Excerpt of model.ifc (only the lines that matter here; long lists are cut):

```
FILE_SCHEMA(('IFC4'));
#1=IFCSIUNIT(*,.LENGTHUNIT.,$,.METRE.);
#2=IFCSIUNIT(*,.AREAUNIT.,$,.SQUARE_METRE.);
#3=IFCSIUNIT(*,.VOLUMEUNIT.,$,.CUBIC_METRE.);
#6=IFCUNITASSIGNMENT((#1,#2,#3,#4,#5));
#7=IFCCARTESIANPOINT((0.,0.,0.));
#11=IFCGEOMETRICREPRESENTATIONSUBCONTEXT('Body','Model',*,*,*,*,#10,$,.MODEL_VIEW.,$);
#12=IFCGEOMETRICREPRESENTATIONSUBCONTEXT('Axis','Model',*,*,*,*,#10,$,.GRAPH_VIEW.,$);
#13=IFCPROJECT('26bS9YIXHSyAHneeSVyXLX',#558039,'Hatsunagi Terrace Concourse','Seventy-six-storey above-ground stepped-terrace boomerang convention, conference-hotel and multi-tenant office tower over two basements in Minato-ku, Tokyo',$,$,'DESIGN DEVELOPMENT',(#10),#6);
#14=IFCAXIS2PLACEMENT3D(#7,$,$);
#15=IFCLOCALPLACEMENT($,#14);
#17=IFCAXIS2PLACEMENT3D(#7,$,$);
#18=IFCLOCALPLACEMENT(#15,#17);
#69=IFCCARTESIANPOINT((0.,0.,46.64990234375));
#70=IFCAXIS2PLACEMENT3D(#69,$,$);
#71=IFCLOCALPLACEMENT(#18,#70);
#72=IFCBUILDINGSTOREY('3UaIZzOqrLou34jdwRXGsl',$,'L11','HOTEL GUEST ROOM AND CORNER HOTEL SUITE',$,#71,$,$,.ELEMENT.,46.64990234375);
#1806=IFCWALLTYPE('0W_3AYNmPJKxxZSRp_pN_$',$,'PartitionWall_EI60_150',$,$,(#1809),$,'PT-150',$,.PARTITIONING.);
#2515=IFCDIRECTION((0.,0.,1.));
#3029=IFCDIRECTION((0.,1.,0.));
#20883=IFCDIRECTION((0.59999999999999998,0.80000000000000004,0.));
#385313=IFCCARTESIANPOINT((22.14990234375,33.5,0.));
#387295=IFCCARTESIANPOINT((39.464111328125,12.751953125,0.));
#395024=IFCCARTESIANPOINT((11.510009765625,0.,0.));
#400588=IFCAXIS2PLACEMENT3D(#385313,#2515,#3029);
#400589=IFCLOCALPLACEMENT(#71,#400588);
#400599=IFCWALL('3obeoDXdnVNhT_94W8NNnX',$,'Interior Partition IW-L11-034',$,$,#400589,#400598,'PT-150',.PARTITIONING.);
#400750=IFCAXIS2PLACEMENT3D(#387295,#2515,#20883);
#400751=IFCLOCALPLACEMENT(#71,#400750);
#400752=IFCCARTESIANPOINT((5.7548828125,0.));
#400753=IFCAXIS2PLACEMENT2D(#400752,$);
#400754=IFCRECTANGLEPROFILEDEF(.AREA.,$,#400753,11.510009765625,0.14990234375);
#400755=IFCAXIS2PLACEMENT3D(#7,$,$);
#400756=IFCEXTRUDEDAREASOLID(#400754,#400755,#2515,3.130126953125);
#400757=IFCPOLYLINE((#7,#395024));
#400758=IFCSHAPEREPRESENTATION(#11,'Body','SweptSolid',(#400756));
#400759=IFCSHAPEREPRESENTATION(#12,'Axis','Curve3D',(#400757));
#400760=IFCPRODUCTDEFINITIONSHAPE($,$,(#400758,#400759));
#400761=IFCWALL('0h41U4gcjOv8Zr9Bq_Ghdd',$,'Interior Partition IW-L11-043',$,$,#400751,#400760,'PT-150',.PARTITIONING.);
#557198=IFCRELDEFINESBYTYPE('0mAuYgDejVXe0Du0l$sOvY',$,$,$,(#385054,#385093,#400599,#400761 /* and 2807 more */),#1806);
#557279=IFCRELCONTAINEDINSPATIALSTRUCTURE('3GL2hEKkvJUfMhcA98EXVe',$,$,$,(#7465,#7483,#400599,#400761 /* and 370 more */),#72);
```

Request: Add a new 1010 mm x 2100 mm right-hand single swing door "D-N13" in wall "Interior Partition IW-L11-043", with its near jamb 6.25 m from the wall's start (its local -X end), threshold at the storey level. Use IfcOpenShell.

```python
import numpy as np
import ifcopenshell
import ifcopenshell.api.feature
import ifcopenshell.api.geometry
import ifcopenshell.api.root
import ifcopenshell.api.spatial
import ifcopenshell.geom
import ifcopenshell.util.element
import ifcopenshell.util.placement
import ifcopenshell.util.representation
import ifcopenshell.util.shape
import ifcopenshell.util.unit

model = ifcopenshell.open("model.ifc")
unit_scale = ifcopenshell.util.unit.calculate_unit_scale(model)
settings = ifcopenshell.geom.settings()


def volume(element):
    """Net volume in cubic metres, openings subtracted."""
    shape = ifcopenshell.geom.create_shape(settings, element)
    return ifcopenshell.util.shape.get_volume(shape.geometry)


wall = model.by_guid("0h41U4gcjOv8Zr9Bq_Ghdd")
storey = ifcopenshell.util.element.get_container(wall, ifc_class="IfcBuildingStorey")
context = ifcopenshell.util.representation.get_context(model, "Model", "Body", "MODEL_VIEW")
before = volume(wall)

width, height, from_end, sill = 1.01, 2.1, 6.25, 0.0  # metres

# The wall runs along its own X axis, and the end named is its -X end.
wall_shape = ifcopenshell.geom.create_shape(settings, wall)
x, y, z = ifcopenshell.util.shape.get_vertices(wall_shape.geometry).T
start = x.min() + from_end
face, thickness = float(y.min()), float(y.max() - y.min())
wall_matrix = ifcopenshell.util.placement.get_local_placement(wall.ObjectPlacement)
level = ifcopenshell.util.placement.get_local_placement(storey.ObjectPlacement)[2, 3]


def in_wall(x, y):
    """Placement at x, y metres in the wall's axes, at sill height."""
    matrix = wall_matrix.copy()
    matrix[:, 3] = wall_matrix @ np.array([x / unit_scale, y / unit_scale, 0.0, 1.0])
    matrix[2, 3] = level + sill / unit_scale
    return matrix


# Opening: a box that overshoots both wall faces by 50 mm.
opening = ifcopenshell.api.root.create_entity(model, ifc_class="IfcOpeningElement", predefined_type="OPENING")
box = ifcopenshell.api.geometry.add_wall_representation(
    model, context=context, length=width, height=height, thickness=thickness + 0.1
)
ifcopenshell.api.geometry.assign_representation(model, product=opening, representation=box)
ifcopenshell.api.geometry.edit_object_placement(model, product=opening, matrix=in_wall(start, face - 0.05), is_si=False)
ifcopenshell.api.feature.add_feature(model, feature=opening, element=wall)

door = ifcopenshell.api.root.create_entity(model, ifc_class="IfcDoor", name="D-N13", predefined_type="DOOR")
door.OverallWidth, door.OverallHeight = width / unit_scale, height / unit_scale
door.OperationType = "SINGLE_SWING_RIGHT"
body = ifcopenshell.api.geometry.add_door_representation(
    model,
    context=context,
    overall_width=door.OverallWidth,
    overall_height=door.OverallHeight,
    operation_type="SINGLE_SWING_RIGHT",
    lining_properties={"LiningDepth": thickness / unit_scale, "ThresholdDepth": thickness / unit_scale},
)
ifcopenshell.api.geometry.assign_representation(model, product=door, representation=body)
ifcopenshell.api.spatial.assign_container(model, products=[door], relating_structure=storey)
ifcopenshell.api.feature.add_filling(model, opening=opening, element=door)

# The lining spans the wall, so the door starts at the wall face.
ifcopenshell.api.geometry.edit_object_placement(model, product=door, matrix=in_wall(start, face), is_si=False)

after = volume(wall)

print(f"wall volume {before:.3f} -> {after:.3f} m3")

model.write("model-out.ifc")
```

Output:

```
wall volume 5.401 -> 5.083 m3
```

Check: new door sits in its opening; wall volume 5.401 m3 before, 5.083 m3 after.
